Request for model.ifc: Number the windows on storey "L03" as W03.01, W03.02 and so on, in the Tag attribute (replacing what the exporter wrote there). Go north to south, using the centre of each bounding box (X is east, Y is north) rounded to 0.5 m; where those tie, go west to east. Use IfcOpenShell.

First a look at what the model holds.

```python
import ifcopenshell
import ifcopenshell.util.element
import ifcopenshell.util.placement

model = ifcopenshell.open("model.ifc")
print(model.schema)
storey = next(s for s in model.by_type("IfcBuildingStorey") if s.Name == "L03")
windows = [e for e in ifcopenshell.util.element.get_decomposition(storey) if e.is_a("IfcWindow")]
for e in sorted(windows, key=lambda e: e.id()):
    origin = ifcopenshell.util.placement.get_local_placement(e.ObjectPlacement)[:3, 3]
    print(e.id(), e.Tag, e.Name, origin.round(2) + 0.0, sep=" | ")
```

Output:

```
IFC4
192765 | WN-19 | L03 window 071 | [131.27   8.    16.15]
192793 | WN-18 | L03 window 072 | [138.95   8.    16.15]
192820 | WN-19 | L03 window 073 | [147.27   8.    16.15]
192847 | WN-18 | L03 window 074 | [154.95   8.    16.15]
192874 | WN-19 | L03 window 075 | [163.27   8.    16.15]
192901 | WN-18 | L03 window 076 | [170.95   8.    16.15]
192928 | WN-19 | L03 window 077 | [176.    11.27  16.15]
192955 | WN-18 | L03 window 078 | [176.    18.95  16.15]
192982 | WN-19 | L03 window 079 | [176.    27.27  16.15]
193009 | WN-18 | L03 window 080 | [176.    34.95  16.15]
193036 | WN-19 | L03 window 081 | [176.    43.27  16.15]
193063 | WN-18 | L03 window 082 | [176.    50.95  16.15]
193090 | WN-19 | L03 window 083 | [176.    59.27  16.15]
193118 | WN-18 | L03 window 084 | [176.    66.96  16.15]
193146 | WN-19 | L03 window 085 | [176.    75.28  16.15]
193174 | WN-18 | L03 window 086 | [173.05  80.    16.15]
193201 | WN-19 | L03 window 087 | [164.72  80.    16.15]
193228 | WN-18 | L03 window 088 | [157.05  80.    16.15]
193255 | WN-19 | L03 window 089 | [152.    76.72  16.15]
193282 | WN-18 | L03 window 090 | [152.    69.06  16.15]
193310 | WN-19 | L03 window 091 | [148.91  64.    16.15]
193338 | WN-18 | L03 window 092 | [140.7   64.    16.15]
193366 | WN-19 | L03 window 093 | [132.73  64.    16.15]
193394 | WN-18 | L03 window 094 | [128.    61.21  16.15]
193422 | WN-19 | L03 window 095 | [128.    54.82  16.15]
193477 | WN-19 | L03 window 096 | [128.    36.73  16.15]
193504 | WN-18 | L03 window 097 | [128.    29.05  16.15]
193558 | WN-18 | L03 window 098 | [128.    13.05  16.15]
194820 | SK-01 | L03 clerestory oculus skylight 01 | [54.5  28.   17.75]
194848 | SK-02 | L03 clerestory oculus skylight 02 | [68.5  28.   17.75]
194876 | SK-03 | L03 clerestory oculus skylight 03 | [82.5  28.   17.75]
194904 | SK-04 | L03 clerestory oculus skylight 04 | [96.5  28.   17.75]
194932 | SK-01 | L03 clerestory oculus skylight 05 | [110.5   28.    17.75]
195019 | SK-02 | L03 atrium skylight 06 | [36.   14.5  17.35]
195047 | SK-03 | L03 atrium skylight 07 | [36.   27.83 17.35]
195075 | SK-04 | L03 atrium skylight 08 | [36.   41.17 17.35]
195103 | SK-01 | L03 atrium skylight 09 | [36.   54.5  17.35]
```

```python
import ifcopenshell
import ifcopenshell.geom
import ifcopenshell.util.element
import ifcopenshell.util.shape

model = ifcopenshell.open("model.ifc")
settings = ifcopenshell.geom.settings()
settings.set("use-world-coords", True)


def centre(element):
    shape = ifcopenshell.geom.create_shape(settings, element)
    return ifcopenshell.util.shape.get_bbox_centroid(shape.geometry)


storey = next(s for s in model.by_type("IfcBuildingStorey") if s.Name == "L03")
windows = [e for e in ifcopenshell.util.element.get_decomposition(storey) if e.is_a("IfcWindow")]

# Insertion points can sit at a corner or the storey origin, so sort by the geometry (in metres).
centres = {e: centre(e) for e in windows}
windows.sort(key=lambda e: (-round(centres[e][1] / 0.5), centres[e][0]))

for i, e in enumerate(windows, start=1):
    number = f"W03.{i:02d}"
    e.Tag = number
    print(e.id(), number)

model.write("model_updated.ifc")
```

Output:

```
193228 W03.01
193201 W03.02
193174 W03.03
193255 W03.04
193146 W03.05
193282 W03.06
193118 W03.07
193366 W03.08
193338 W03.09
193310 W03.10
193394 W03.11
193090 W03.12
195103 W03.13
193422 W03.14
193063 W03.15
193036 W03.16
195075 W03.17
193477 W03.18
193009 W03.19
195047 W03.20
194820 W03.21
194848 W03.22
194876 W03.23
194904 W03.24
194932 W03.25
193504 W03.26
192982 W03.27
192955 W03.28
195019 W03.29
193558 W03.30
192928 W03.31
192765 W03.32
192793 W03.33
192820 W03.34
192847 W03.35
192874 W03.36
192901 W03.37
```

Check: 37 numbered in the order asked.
